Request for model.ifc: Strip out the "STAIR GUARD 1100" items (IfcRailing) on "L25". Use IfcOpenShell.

First a look at what the model holds.

```python
import ifcopenshell
import ifcopenshell.util.element

model = ifcopenshell.open("model.ifc")
print(model.schema)
storey = next(s for s in model.by_type("IfcBuildingStorey") if s.Name == "L25")
railings = [e for e in ifcopenshell.util.element.get_decomposition(storey) if e.is_a("IfcRailing")]
seen = {}
for e in railings:
    element_type = ifcopenshell.util.element.get_type(e)
    name = element_type.Name if element_type not in (None, e) else None
    seen[name] = seen.get(name, 0) + 1
for name, count in sorted(seen.items(), key=str):
    print(count, "x", name)
```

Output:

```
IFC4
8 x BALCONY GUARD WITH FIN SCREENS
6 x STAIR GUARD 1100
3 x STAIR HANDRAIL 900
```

```python
import ifcopenshell
import ifcopenshell.api.root
import ifcopenshell.util.element

model = ifcopenshell.open("model.ifc")

storey = next(s for s in model.by_type("IfcBuildingStorey") if s.Name == "L25")
railings = [e for e in ifcopenshell.util.element.get_decomposition(storey) if e.is_a("IfcRailing")]
targets = [e for e in railings if (t := ifcopenshell.util.element.get_type(e)) not in (None, e) and t.Name == "STAIR GUARD 1100"]

for e in targets:
    ifcopenshell.api.root.remove_product(model, product=e)
print(len(targets), "removed")

model.write("model-out.ifc")
```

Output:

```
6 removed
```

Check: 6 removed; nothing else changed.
